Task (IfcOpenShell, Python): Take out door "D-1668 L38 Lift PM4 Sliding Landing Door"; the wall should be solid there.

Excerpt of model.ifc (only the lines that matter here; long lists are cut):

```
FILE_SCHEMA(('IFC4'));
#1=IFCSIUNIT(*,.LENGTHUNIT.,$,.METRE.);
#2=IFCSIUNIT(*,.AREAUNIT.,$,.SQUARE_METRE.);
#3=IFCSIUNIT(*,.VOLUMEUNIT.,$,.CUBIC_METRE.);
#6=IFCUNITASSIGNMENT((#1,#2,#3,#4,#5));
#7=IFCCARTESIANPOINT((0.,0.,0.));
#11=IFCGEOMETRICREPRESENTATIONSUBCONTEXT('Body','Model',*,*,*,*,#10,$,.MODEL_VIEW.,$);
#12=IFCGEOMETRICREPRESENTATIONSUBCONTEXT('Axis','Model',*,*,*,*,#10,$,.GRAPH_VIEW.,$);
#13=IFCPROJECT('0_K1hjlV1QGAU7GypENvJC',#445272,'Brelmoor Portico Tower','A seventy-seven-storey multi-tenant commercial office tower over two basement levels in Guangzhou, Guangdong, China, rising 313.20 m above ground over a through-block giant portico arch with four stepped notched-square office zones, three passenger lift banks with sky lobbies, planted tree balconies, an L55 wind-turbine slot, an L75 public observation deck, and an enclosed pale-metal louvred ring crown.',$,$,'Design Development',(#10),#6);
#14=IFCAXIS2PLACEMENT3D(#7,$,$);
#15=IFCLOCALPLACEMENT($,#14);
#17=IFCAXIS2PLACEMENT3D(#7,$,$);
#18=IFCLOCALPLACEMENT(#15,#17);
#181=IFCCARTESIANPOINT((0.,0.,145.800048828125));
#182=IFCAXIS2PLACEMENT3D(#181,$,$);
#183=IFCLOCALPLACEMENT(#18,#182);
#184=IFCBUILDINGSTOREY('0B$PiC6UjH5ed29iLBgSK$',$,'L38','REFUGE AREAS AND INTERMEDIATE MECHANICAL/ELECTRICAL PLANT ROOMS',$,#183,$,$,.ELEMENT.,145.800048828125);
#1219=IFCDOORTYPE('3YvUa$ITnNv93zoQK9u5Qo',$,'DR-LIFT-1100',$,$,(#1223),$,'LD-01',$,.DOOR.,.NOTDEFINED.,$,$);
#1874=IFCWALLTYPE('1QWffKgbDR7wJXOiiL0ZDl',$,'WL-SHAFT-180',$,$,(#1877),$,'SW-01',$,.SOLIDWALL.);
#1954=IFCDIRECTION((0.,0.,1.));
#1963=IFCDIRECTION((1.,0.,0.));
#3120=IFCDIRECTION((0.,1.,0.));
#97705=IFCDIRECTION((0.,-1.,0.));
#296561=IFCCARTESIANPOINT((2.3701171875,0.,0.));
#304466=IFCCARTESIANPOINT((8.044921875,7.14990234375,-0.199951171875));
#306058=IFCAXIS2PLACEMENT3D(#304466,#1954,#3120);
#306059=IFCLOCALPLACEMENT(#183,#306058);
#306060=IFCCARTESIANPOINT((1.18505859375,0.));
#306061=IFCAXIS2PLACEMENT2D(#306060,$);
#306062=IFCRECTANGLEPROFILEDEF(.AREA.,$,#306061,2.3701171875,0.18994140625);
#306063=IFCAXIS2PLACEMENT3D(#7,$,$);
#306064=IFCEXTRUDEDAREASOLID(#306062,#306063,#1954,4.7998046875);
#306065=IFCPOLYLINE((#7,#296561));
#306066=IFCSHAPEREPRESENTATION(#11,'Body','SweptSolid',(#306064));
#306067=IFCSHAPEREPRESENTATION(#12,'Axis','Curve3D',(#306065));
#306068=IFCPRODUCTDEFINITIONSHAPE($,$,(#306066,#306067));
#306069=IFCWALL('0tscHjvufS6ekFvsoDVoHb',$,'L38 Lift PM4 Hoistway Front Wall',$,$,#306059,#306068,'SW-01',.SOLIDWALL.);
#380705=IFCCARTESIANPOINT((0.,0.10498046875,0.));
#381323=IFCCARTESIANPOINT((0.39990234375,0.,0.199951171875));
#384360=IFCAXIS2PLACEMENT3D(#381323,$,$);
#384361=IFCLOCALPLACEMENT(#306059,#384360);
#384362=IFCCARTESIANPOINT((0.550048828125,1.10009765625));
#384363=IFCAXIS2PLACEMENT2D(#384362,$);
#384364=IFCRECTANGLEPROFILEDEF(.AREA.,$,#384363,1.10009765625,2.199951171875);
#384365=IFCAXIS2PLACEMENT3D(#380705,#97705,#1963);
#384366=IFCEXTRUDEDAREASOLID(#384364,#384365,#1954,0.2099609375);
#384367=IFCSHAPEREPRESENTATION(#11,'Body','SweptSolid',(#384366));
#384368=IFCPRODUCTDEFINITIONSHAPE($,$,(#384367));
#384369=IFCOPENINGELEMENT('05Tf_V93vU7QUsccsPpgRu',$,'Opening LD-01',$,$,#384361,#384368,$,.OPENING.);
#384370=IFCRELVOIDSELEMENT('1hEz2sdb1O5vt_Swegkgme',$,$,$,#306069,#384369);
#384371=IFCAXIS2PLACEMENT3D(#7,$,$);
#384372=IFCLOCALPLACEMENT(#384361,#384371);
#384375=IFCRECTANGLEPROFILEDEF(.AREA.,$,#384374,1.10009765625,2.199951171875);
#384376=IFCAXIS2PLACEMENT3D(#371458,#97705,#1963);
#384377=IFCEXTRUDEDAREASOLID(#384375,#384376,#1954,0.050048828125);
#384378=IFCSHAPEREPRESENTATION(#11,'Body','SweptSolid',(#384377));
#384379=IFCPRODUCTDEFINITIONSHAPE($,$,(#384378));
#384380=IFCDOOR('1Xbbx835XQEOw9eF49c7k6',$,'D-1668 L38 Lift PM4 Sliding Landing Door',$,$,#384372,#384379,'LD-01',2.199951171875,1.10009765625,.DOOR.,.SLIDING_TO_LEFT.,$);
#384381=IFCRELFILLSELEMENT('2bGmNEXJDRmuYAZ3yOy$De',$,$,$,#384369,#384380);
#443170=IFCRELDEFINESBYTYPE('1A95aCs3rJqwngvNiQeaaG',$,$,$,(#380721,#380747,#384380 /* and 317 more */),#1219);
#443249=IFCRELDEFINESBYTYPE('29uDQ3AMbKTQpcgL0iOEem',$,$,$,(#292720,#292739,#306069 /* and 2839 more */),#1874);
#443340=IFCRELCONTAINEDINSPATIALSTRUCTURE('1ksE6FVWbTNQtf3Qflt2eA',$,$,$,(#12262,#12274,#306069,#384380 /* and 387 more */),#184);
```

```python
import ifcopenshell
import ifcopenshell.api.feature
import ifcopenshell.api.root
import ifcopenshell.geom
import ifcopenshell.util.shape

model = ifcopenshell.open("model.ifc")
settings = ifcopenshell.geom.settings()


def volume(element):
    """Net volume in cubic metres, openings subtracted."""
    shape = ifcopenshell.geom.create_shape(settings, element)
    return ifcopenshell.util.shape.get_volume(shape.geometry)


door = model.by_guid("1Xbbx835XQEOw9eF49c7k6")
opening = door.FillsVoids[0].RelatingOpeningElement
wall = opening.VoidsElements[0].RelatingBuildingElement
before = volume(wall)

ifcopenshell.api.root.remove_product(model, product=door)
ifcopenshell.api.feature.remove_feature(model, feature=opening)

after = volume(wall)

print(f"wall volume {before:.3f} -> {after:.3f} m3")

model.write("model_updated.ifc")
```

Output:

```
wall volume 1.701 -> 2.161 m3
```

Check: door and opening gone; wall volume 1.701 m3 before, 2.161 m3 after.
